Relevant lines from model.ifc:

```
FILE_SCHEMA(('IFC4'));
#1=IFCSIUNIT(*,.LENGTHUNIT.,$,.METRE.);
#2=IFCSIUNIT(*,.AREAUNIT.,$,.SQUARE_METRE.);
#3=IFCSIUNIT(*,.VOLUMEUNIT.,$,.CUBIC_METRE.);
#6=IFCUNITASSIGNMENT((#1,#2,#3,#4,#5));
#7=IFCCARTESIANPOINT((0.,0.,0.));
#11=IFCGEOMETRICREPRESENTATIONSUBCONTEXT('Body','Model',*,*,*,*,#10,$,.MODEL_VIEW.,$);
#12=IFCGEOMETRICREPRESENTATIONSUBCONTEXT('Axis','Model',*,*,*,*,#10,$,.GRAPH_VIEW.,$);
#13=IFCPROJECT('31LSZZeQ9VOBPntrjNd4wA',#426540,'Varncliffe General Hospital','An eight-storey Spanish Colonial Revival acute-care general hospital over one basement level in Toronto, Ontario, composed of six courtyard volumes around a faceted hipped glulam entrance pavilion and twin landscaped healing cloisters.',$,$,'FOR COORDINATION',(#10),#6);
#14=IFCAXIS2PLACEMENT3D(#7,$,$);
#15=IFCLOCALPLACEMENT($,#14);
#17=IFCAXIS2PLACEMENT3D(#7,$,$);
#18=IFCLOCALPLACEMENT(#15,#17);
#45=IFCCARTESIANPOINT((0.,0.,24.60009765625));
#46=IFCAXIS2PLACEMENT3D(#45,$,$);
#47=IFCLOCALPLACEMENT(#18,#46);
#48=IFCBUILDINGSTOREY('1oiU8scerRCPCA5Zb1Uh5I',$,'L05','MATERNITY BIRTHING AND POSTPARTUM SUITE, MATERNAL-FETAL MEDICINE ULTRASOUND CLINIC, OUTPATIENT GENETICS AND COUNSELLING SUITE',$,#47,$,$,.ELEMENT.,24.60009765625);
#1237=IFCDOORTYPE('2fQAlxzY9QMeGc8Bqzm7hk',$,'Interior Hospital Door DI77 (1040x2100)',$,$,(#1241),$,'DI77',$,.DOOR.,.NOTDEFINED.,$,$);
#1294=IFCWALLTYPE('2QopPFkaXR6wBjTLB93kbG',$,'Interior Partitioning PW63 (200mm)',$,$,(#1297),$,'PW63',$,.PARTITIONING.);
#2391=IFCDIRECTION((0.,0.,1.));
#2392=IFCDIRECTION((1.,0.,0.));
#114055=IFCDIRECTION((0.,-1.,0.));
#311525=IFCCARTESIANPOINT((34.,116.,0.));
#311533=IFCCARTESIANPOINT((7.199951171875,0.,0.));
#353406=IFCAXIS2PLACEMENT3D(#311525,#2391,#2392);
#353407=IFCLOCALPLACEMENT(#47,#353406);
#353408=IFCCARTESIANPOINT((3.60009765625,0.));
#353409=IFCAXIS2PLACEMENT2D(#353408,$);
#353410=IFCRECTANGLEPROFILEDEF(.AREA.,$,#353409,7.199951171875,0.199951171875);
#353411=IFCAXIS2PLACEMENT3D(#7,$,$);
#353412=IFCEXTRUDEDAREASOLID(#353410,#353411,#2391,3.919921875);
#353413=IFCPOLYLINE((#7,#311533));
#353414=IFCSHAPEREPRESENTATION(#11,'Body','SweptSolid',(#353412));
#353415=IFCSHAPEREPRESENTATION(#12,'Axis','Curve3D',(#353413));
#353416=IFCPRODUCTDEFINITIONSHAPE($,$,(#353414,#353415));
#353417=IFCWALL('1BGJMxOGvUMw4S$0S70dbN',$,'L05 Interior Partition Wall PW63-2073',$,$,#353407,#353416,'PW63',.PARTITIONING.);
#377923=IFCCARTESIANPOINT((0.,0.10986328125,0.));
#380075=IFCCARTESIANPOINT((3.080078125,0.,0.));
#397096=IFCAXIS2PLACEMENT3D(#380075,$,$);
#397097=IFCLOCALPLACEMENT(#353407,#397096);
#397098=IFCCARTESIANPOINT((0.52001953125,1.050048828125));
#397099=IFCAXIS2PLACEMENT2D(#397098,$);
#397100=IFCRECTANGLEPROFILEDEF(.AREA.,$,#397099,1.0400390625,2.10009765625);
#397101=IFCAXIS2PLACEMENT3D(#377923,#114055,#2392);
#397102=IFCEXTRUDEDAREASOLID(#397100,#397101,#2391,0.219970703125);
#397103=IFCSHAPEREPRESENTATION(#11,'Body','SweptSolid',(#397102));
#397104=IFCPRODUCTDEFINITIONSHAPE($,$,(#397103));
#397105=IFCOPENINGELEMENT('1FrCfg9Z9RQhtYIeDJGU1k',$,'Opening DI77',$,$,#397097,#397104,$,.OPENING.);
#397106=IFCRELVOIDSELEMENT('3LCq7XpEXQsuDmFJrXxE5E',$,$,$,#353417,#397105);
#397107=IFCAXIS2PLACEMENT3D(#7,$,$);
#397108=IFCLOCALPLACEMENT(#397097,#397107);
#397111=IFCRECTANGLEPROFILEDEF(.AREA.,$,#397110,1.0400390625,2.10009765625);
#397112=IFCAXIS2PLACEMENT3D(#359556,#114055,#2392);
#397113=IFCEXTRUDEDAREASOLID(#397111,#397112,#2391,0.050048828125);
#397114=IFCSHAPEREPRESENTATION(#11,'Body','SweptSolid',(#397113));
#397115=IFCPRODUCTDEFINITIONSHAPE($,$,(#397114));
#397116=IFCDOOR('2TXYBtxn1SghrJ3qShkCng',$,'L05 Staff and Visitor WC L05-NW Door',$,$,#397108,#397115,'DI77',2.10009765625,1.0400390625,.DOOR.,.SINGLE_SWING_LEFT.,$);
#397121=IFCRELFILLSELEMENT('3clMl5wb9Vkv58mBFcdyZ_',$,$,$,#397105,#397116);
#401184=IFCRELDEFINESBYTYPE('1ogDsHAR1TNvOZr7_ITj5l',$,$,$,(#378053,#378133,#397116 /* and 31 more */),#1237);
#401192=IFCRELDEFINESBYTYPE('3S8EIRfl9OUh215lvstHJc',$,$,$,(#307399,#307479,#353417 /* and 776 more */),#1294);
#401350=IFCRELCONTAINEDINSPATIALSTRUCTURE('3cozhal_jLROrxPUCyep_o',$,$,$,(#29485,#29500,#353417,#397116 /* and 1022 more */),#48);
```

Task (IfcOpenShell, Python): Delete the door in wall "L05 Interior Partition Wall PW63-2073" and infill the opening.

```python
import ifcopenshell
import ifcopenshell.api.feature
import ifcopenshell.api.root
import ifcopenshell.geom
import ifcopenshell.util.shape

model = ifcopenshell.open("model.ifc")
settings = ifcopenshell.geom.settings()


def volume(element):
    """Net volume in cubic metres, openings subtracted."""
    shape = ifcopenshell.geom.create_shape(settings, element)
    return ifcopenshell.util.shape.get_volume(shape.geometry)


door = model.by_guid("2TXYBtxn1SghrJ3qShkCng")
opening = door.FillsVoids[0].RelatingOpeningElement
wall = opening.VoidsElements[0].RelatingBuildingElement
before = volume(wall)

ifcopenshell.api.root.remove_product(model, product=door)
ifcopenshell.api.feature.remove_feature(model, feature=opening)

after = volume(wall)

print(f"wall volume {before:.3f} -> {after:.3f} m3")

model.write("model_edited.ifc")
```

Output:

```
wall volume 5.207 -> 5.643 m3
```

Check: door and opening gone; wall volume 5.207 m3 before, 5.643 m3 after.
